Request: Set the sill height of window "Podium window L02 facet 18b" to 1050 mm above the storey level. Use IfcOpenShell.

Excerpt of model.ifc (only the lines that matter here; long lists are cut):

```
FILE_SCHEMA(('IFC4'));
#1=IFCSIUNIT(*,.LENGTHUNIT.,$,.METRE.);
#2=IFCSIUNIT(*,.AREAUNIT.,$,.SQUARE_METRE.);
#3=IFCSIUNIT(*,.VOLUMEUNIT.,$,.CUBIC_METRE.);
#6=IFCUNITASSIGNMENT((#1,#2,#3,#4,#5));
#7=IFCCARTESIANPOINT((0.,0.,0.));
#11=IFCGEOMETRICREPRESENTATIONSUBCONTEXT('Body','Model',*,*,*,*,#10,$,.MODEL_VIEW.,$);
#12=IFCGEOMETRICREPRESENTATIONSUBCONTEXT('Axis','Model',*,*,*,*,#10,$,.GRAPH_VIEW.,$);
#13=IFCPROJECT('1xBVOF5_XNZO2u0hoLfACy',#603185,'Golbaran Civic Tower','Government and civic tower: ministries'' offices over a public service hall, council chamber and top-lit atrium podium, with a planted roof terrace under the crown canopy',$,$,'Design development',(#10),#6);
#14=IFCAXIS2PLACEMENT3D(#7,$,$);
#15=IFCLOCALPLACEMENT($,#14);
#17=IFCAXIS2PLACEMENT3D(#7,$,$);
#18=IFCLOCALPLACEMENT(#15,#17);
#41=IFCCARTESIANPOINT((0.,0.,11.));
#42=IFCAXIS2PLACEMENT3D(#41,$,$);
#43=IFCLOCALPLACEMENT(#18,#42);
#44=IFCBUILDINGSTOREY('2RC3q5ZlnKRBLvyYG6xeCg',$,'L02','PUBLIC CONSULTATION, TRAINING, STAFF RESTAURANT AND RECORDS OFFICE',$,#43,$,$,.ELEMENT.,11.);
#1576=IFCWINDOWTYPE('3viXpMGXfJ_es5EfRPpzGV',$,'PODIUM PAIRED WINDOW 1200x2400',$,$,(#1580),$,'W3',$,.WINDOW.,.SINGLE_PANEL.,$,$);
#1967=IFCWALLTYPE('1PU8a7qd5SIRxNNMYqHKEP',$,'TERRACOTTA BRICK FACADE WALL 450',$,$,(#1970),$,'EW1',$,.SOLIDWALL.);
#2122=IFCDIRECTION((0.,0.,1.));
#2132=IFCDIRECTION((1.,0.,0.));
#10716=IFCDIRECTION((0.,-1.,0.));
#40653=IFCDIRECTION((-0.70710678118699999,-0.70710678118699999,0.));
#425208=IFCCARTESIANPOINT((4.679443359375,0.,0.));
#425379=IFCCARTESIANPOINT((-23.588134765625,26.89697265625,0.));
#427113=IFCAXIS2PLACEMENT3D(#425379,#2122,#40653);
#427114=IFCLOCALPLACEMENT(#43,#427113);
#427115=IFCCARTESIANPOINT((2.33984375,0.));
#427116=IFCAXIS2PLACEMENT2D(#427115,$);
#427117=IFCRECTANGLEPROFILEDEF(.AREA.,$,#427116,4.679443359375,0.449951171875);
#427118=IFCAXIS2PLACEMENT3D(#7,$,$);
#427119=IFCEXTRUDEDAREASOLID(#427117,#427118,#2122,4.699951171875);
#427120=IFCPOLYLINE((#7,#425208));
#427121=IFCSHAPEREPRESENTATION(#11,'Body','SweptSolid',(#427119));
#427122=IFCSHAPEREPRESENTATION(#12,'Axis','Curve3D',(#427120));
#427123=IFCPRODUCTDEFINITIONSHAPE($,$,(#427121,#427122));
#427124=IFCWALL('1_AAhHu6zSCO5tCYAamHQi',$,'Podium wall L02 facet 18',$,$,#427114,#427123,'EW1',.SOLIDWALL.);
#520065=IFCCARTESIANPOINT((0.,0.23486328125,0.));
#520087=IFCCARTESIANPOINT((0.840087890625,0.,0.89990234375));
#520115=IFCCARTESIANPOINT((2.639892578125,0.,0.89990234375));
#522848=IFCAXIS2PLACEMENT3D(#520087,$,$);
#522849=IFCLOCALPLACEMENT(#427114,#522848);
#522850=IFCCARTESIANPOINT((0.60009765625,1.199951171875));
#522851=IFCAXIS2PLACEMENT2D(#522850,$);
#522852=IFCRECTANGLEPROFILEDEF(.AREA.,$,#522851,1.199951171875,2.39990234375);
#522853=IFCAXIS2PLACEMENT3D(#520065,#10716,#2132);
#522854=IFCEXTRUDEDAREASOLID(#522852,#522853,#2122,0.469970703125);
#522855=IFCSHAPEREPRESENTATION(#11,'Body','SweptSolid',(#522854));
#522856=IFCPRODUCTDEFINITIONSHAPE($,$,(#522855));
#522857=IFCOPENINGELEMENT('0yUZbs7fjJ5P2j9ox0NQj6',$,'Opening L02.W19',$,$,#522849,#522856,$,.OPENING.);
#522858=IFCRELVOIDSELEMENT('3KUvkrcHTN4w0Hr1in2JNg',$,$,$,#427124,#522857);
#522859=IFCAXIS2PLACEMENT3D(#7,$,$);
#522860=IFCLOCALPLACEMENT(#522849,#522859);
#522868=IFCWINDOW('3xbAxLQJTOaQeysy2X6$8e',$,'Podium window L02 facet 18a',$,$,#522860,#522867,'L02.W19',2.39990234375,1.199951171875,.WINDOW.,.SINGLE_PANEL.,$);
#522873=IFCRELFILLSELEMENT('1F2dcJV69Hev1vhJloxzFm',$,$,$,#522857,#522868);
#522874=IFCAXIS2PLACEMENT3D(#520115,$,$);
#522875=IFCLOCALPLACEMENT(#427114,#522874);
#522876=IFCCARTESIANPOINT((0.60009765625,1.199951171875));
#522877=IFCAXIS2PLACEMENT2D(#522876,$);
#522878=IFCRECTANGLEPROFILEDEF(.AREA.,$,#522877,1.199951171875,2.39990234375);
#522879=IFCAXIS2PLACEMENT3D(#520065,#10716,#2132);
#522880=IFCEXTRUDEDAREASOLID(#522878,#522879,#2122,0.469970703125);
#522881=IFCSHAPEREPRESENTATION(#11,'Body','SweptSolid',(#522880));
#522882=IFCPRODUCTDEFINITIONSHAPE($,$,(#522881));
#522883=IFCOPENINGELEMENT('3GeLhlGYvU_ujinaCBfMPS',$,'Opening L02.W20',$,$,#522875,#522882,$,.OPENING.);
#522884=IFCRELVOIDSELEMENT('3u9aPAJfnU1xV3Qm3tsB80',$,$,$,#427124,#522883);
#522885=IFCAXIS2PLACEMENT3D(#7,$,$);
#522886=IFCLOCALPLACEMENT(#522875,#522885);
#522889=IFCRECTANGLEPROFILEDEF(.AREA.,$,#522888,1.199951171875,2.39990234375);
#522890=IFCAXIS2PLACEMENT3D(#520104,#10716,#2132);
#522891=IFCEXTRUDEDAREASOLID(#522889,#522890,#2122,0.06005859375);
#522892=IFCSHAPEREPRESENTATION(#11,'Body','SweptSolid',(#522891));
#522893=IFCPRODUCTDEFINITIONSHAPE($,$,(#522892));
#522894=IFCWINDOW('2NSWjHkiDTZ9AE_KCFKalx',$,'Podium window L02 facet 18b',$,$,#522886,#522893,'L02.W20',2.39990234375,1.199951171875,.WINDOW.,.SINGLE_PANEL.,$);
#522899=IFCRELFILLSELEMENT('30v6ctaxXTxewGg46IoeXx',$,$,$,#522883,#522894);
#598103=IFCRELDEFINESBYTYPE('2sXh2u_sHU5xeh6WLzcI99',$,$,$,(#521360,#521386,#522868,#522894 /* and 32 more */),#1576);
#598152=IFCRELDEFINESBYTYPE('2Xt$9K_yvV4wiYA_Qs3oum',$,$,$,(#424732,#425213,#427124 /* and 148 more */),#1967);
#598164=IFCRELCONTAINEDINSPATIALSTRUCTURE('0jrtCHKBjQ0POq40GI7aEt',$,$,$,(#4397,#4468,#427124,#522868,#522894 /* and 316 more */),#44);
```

```python
import numpy as np
import ifcopenshell
import ifcopenshell.api.geometry
import ifcopenshell.geom
import ifcopenshell.util.element
import ifcopenshell.util.placement
import ifcopenshell.util.shape
import ifcopenshell.util.unit

model = ifcopenshell.open("model.ifc")
unit_scale = ifcopenshell.util.unit.calculate_unit_scale(model)

window = model.by_guid("2NSWjHkiDTZ9AE_KCFKalx")
opening = window.FillsVoids[0].RelatingOpeningElement
storey = ifcopenshell.util.element.get_container(window, ifc_class="IfcBuildingStorey")
level = ifcopenshell.util.placement.get_local_placement(storey.ObjectPlacement)[2, 3]

# The opening's origin need not be at the sill, so measure its lowest point.
shape = ifcopenshell.geom.create_shape(ifcopenshell.geom.settings(), opening)
bottom = ifcopenshell.util.shape.get_shape_bottom_elevation(shape, shape.geometry) / unit_scale
dz = level + 1.05 - bottom

shift = np.array([0.0, 0.0, dz])
# The window is placed relative to its opening, so it follows when the opening moves.
matrix = ifcopenshell.util.placement.get_local_placement(opening.ObjectPlacement)
matrix[:3, 3] += shift
ifcopenshell.api.geometry.edit_object_placement(
    model, product=opening, matrix=matrix, is_si=False, should_transform_children=True
)

print(f"moved by {dz * unit_scale:+.3f} m")

model.write("model_updated.ifc")
```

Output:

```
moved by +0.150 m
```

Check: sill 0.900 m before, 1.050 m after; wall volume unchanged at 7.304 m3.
